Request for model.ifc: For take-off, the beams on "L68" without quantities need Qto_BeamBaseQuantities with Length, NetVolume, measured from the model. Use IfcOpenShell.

First a look at what the model holds.

```python
import ifcopenshell
import ifcopenshell.util.element
import ifcopenshell.util.unit

model = ifcopenshell.open("model.ifc")
print(model.schema)
for unit_type in ("LENGTHUNIT", "AREAUNIT", "VOLUMEUNIT"):
    print(unit_type, ifcopenshell.util.unit.calculate_unit_scale(model, unit_type))
storey = next(s for s in model.by_type("IfcBuildingStorey") if s.Name == "L68")
beams = [e for e in ifcopenshell.util.element.get_decomposition(storey) if e.is_a("IfcBeam")]
for e in sorted(beams, key=lambda e: e.id()):
    print(e.id(), e.is_a(), e.Name, list(ifcopenshell.util.element.get_psets(e, qtos_only=True)), sep=" | ")
```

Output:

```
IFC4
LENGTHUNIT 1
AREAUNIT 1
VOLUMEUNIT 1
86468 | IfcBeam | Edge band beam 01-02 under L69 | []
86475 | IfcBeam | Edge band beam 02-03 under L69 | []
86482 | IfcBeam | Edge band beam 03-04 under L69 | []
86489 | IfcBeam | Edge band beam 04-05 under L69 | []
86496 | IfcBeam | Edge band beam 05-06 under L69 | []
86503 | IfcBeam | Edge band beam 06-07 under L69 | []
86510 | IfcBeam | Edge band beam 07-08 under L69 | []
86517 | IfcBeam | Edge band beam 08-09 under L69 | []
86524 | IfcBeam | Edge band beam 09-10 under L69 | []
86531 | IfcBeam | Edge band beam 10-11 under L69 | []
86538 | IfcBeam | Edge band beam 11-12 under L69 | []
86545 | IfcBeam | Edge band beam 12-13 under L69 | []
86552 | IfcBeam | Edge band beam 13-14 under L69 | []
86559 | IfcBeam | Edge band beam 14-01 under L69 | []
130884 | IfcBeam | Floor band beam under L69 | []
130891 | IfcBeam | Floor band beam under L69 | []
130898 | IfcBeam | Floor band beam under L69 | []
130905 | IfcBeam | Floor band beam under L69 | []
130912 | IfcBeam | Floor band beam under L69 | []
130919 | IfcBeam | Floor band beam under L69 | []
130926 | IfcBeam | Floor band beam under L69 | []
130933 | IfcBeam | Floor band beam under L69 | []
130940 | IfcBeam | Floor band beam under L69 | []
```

```python
import ifcopenshell
import ifcopenshell.api.pset
import ifcopenshell.geom
import ifcopenshell.util.element
import ifcopenshell.util.shape
import ifcopenshell.util.unit

model = ifcopenshell.open("model.ifc")
unit_scale = ifcopenshell.util.unit.calculate_unit_scale(model)
volume_scale = ifcopenshell.util.unit.calculate_unit_scale(model, "VOLUMEUNIT")
settings = ifcopenshell.geom.settings()

storey = next(s for s in model.by_type("IfcBuildingStorey") if s.Name == "L68")
beams = [e for e in ifcopenshell.util.element.get_decomposition(storey) if e.is_a("IfcBeam")]

for e in sorted(beams, key=lambda e: e.id()):
    if ifcopenshell.util.element.get_psets(e, qtos_only=True, should_inherit=False):
        continue
    # Geometry comes back in metres, in the element's own axes.
    shape = ifcopenshell.geom.create_shape(settings, e)
    values = {
        "Length": ifcopenshell.util.shape.get_max_xyz(shape.geometry) / unit_scale,
        "NetVolume": ifcopenshell.util.shape.get_volume(shape.geometry) / volume_scale,
    }
    qto = ifcopenshell.api.pset.add_qto(model, product=e, name="Qto_BeamBaseQuantities")
    ifcopenshell.api.pset.edit_qto(model, qto=qto, properties=values)
    print(e.id(), {k: round(v, 3) for k, v in values.items()})

model.write("model-out.ifc")
```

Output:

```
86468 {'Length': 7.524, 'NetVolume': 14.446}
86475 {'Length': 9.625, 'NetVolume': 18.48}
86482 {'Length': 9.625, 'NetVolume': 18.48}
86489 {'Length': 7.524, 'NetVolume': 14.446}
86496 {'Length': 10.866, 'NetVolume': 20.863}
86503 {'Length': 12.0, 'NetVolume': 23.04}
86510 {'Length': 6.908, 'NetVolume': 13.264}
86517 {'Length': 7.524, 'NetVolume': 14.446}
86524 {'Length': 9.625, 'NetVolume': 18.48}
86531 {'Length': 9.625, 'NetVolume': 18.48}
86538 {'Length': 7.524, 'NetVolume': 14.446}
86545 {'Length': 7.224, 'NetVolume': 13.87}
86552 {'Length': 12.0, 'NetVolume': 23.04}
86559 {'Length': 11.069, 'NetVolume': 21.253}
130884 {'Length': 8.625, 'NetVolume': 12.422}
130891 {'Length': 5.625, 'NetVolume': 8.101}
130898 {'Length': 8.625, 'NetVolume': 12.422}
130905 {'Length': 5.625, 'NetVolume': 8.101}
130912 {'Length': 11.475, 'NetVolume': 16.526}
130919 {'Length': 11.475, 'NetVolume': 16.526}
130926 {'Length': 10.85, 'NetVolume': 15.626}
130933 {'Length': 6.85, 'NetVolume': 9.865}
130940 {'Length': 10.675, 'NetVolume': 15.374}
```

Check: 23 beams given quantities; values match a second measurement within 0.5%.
